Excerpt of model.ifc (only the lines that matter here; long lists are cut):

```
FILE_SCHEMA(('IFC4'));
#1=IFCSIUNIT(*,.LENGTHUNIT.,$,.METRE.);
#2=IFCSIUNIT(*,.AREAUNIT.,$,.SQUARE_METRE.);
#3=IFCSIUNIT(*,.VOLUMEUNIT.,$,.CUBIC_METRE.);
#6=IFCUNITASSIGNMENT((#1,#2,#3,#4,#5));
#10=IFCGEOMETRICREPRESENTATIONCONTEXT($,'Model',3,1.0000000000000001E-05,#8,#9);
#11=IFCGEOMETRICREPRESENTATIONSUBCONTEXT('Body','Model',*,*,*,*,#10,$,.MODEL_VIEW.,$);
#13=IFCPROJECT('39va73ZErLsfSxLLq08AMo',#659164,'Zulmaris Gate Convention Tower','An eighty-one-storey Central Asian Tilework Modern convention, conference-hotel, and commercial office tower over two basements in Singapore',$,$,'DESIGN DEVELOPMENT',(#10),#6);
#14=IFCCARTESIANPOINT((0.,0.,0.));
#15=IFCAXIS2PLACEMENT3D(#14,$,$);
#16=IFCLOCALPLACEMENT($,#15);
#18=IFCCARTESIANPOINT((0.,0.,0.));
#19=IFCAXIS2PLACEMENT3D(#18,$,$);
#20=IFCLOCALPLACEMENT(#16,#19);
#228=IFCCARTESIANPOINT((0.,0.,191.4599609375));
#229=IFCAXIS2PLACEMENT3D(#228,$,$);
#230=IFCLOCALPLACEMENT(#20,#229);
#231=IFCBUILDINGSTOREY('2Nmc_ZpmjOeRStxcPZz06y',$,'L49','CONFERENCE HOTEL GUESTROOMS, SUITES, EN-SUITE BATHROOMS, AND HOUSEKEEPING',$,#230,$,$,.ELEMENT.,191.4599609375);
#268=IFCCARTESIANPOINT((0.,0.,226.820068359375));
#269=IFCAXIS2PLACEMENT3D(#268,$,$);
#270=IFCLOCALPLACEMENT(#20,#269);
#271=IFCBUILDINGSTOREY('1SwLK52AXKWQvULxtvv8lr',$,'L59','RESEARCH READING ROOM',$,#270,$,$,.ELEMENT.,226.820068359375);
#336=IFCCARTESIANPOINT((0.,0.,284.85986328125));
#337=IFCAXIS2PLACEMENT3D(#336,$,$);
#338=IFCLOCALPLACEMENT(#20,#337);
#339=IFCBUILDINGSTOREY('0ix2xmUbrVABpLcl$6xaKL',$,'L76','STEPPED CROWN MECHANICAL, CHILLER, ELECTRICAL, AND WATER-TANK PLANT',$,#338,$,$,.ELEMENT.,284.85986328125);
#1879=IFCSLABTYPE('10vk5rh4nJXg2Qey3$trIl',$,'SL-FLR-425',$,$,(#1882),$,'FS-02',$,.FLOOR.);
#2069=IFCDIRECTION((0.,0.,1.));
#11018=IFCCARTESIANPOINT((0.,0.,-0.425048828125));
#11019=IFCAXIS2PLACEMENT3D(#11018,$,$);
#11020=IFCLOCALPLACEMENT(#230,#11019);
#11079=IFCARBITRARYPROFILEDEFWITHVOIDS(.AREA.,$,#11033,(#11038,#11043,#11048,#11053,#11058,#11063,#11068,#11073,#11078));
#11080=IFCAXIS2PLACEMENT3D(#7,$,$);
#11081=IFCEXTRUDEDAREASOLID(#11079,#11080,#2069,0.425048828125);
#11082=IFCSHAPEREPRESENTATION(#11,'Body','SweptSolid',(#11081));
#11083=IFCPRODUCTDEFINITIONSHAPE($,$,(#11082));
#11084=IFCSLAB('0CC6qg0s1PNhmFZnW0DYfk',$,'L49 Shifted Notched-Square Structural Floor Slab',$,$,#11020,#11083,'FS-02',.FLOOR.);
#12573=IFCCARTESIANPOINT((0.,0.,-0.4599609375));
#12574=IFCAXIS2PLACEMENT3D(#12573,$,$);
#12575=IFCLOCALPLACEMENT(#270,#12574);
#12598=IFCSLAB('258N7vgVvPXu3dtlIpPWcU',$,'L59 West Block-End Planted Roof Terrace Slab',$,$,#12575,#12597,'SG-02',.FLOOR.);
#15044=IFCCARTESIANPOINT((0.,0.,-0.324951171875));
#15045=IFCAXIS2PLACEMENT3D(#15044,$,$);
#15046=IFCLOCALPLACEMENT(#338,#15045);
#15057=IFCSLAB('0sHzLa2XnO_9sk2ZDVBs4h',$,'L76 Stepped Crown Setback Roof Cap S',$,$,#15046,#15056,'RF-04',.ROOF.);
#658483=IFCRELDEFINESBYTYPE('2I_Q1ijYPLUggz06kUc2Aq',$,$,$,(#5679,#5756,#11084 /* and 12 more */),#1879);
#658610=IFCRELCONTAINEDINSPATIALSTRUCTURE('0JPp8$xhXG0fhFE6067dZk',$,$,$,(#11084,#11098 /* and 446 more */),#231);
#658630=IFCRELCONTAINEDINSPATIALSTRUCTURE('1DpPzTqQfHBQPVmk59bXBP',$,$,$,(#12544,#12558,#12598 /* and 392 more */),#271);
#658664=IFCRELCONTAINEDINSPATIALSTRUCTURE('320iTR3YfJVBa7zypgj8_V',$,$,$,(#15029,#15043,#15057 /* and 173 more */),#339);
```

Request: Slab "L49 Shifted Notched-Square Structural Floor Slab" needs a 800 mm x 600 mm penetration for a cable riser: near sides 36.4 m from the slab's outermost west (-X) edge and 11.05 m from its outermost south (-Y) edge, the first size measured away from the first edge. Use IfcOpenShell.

```python
import numpy as np
import ifcopenshell
import ifcopenshell.api.feature
import ifcopenshell.api.geometry
import ifcopenshell.api.root
import ifcopenshell.geom
import ifcopenshell.util.placement
import ifcopenshell.util.representation
import ifcopenshell.util.shape
import ifcopenshell.util.unit

model = ifcopenshell.open("model.ifc")
unit_scale = ifcopenshell.util.unit.calculate_unit_scale(model)
settings = ifcopenshell.geom.settings()


def volume(element):
    """Net volume in cubic metres, openings subtracted."""
    shape = ifcopenshell.geom.create_shape(settings, element)
    return ifcopenshell.util.shape.get_volume(shape.geometry)


slab = model.by_guid("0CC6qg0s1PNhmFZnW0DYfk")
before = volume(slab)

# Extent in the slab's own axes, in metres. The edges named are its -X and -Y sides.
slab_shape = ifcopenshell.geom.create_shape(settings, slab)
vertices = ifcopenshell.util.shape.get_vertices(slab_shape.geometry)
x_min, y_min, bottom = vertices.min(axis=0)
top = vertices[:, 2].max()

opening = ifcopenshell.api.root.create_entity(model, ifc_class="IfcOpeningElement", name="Cable riser opening", predefined_type="OPENING")
context = ifcopenshell.util.representation.get_context(model, "Model", "Body", "MODEL_VIEW")
width, depth = 0.8, 0.6
outline = [(0.0, 0.0), (width, 0.0), (width, depth), (0.0, depth), (0.0, 0.0)]
# Overshoot both faces by 50 mm so the cut is clean.
shape = ifcopenshell.api.geometry.add_slab_representation(
    model, context=context, depth=top - bottom + 0.1, polyline=outline
)
ifcopenshell.api.geometry.assign_representation(model, product=opening, representation=shape)

matrix = ifcopenshell.util.placement.get_local_placement(slab.ObjectPlacement)
matrix[:, 3] = matrix @ np.append(np.array([x_min + 36.4, y_min + 11.05, bottom - 0.05]) / unit_scale, 1.0)
ifcopenshell.api.geometry.edit_object_placement(model, product=opening, matrix=matrix, is_si=False)
ifcopenshell.api.feature.add_feature(model, feature=opening, element=slab)

after = volume(slab)

print(f"slab volume {before:.3f} -> {after:.3f} m3")

model.write("model-out.ifc")
```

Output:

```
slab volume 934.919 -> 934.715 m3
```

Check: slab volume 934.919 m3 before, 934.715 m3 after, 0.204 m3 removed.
